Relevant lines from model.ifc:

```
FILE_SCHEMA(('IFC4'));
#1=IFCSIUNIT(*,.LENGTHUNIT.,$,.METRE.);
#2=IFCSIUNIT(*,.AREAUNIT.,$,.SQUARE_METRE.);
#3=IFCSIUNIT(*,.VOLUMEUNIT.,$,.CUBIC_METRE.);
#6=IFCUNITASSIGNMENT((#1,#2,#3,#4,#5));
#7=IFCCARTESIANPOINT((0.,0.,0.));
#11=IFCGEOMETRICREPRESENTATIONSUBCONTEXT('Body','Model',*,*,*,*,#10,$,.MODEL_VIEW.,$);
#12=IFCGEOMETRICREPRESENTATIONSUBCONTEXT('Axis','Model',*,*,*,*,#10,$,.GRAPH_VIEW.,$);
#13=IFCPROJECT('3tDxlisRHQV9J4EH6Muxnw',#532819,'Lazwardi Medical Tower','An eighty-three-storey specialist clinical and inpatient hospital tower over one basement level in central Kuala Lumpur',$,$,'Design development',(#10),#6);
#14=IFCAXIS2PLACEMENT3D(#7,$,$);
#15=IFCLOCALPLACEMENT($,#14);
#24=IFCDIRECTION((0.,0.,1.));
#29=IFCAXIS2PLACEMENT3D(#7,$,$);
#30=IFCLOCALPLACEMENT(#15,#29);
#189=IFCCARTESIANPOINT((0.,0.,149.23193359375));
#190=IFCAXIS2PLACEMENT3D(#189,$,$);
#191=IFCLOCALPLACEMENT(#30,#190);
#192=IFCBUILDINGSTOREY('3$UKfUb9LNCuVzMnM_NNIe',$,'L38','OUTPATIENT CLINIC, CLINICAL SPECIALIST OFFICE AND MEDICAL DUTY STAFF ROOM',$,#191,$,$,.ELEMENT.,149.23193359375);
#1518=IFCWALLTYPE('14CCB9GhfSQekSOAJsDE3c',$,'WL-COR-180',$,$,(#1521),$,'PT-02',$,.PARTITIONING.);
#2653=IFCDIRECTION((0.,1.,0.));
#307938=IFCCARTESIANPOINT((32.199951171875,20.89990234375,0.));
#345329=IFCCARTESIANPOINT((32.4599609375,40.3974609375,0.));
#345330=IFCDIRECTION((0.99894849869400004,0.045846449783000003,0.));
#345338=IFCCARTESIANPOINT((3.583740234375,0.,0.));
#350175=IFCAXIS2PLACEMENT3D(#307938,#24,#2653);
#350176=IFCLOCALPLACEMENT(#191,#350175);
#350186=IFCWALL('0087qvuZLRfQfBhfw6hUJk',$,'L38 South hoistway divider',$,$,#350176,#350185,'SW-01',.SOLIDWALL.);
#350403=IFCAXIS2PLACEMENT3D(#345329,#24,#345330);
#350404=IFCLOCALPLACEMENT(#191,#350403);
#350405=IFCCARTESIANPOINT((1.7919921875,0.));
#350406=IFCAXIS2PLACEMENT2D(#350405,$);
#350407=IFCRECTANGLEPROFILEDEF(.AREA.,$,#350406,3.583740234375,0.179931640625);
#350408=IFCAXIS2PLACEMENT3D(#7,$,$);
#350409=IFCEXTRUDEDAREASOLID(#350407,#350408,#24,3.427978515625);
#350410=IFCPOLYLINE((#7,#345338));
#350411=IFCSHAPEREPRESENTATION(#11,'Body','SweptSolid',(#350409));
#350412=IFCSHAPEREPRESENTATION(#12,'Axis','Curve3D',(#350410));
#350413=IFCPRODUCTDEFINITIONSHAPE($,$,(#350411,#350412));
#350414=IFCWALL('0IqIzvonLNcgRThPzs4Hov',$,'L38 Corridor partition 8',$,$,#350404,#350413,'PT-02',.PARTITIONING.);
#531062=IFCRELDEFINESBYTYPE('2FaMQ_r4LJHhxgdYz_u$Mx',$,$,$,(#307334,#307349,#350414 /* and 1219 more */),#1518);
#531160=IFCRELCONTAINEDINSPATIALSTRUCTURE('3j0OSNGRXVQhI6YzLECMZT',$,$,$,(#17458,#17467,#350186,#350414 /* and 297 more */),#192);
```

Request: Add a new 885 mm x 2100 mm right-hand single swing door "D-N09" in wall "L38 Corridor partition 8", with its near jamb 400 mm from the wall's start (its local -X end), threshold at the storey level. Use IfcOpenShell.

```python
import numpy as np
import ifcopenshell
import ifcopenshell.api.feature
import ifcopenshell.api.geometry
import ifcopenshell.api.root
import ifcopenshell.api.spatial
import ifcopenshell.geom
import ifcopenshell.util.element
import ifcopenshell.util.placement
import ifcopenshell.util.representation
import ifcopenshell.util.shape
import ifcopenshell.util.unit

model = ifcopenshell.open("model.ifc")
unit_scale = ifcopenshell.util.unit.calculate_unit_scale(model)
settings = ifcopenshell.geom.settings()


def volume(element):
    """Net volume in cubic metres, openings subtracted."""
    shape = ifcopenshell.geom.create_shape(settings, element)
    return ifcopenshell.util.shape.get_volume(shape.geometry)


wall = model.by_guid("0IqIzvonLNcgRThPzs4Hov")
storey = ifcopenshell.util.element.get_container(wall, ifc_class="IfcBuildingStorey")
context = ifcopenshell.util.representation.get_context(model, "Model", "Body", "MODEL_VIEW")
before = volume(wall)

width, height, from_end, sill = 0.885, 2.1, 0.4, 0.0  # metres

# The wall runs along its own X axis, and the end named is its -X end.
wall_shape = ifcopenshell.geom.create_shape(settings, wall)
x, y, z = ifcopenshell.util.shape.get_vertices(wall_shape.geometry).T
start = x.min() + from_end
face, thickness = float(y.min()), float(y.max() - y.min())
wall_matrix = ifcopenshell.util.placement.get_local_placement(wall.ObjectPlacement)
level = ifcopenshell.util.placement.get_local_placement(storey.ObjectPlacement)[2, 3]


def in_wall(x, y):
    """Placement at x, y metres in the wall's axes, at sill height."""
    matrix = wall_matrix.copy()
    matrix[:, 3] = wall_matrix @ np.array([x / unit_scale, y / unit_scale, 0.0, 1.0])
    matrix[2, 3] = level + sill / unit_scale
    return matrix


# Opening: a box that overshoots both wall faces by 50 mm.
opening = ifcopenshell.api.root.create_entity(model, ifc_class="IfcOpeningElement", predefined_type="OPENING")
box = ifcopenshell.api.geometry.add_wall_representation(
    model, context=context, length=width, height=height, thickness=thickness + 0.1
)
ifcopenshell.api.geometry.assign_representation(model, product=opening, representation=box)
ifcopenshell.api.geometry.edit_object_placement(model, product=opening, matrix=in_wall(start, face - 0.05), is_si=False)
ifcopenshell.api.feature.add_feature(model, feature=opening, element=wall)

door = ifcopenshell.api.root.create_entity(model, ifc_class="IfcDoor", name="D-N09", predefined_type="DOOR")
door.OverallWidth, door.OverallHeight = width / unit_scale, height / unit_scale
door.OperationType = "SINGLE_SWING_RIGHT"
body = ifcopenshell.api.geometry.add_door_representation(
    model,
    context=context,
    overall_width=door.OverallWidth,
    overall_height=door.OverallHeight,
    operation_type="SINGLE_SWING_RIGHT",
    lining_properties={"LiningDepth": thickness / unit_scale, "ThresholdDepth": thickness / unit_scale},
)
ifcopenshell.api.geometry.assign_representation(model, product=door, representation=body)
ifcopenshell.api.spatial.assign_container(model, products=[door], relating_structure=storey)
ifcopenshell.api.feature.add_filling(model, opening=opening, element=door)

# The lining spans the wall, so the door starts at the wall face.
ifcopenshell.api.geometry.edit_object_placement(model, product=door, matrix=in_wall(start, face), is_si=False)

after = volume(wall)

print(f"wall volume {before:.3f} -> {after:.3f} m3")

model.write("model_rev.ifc")
```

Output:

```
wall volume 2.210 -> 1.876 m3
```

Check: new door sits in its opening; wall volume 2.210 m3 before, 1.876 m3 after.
